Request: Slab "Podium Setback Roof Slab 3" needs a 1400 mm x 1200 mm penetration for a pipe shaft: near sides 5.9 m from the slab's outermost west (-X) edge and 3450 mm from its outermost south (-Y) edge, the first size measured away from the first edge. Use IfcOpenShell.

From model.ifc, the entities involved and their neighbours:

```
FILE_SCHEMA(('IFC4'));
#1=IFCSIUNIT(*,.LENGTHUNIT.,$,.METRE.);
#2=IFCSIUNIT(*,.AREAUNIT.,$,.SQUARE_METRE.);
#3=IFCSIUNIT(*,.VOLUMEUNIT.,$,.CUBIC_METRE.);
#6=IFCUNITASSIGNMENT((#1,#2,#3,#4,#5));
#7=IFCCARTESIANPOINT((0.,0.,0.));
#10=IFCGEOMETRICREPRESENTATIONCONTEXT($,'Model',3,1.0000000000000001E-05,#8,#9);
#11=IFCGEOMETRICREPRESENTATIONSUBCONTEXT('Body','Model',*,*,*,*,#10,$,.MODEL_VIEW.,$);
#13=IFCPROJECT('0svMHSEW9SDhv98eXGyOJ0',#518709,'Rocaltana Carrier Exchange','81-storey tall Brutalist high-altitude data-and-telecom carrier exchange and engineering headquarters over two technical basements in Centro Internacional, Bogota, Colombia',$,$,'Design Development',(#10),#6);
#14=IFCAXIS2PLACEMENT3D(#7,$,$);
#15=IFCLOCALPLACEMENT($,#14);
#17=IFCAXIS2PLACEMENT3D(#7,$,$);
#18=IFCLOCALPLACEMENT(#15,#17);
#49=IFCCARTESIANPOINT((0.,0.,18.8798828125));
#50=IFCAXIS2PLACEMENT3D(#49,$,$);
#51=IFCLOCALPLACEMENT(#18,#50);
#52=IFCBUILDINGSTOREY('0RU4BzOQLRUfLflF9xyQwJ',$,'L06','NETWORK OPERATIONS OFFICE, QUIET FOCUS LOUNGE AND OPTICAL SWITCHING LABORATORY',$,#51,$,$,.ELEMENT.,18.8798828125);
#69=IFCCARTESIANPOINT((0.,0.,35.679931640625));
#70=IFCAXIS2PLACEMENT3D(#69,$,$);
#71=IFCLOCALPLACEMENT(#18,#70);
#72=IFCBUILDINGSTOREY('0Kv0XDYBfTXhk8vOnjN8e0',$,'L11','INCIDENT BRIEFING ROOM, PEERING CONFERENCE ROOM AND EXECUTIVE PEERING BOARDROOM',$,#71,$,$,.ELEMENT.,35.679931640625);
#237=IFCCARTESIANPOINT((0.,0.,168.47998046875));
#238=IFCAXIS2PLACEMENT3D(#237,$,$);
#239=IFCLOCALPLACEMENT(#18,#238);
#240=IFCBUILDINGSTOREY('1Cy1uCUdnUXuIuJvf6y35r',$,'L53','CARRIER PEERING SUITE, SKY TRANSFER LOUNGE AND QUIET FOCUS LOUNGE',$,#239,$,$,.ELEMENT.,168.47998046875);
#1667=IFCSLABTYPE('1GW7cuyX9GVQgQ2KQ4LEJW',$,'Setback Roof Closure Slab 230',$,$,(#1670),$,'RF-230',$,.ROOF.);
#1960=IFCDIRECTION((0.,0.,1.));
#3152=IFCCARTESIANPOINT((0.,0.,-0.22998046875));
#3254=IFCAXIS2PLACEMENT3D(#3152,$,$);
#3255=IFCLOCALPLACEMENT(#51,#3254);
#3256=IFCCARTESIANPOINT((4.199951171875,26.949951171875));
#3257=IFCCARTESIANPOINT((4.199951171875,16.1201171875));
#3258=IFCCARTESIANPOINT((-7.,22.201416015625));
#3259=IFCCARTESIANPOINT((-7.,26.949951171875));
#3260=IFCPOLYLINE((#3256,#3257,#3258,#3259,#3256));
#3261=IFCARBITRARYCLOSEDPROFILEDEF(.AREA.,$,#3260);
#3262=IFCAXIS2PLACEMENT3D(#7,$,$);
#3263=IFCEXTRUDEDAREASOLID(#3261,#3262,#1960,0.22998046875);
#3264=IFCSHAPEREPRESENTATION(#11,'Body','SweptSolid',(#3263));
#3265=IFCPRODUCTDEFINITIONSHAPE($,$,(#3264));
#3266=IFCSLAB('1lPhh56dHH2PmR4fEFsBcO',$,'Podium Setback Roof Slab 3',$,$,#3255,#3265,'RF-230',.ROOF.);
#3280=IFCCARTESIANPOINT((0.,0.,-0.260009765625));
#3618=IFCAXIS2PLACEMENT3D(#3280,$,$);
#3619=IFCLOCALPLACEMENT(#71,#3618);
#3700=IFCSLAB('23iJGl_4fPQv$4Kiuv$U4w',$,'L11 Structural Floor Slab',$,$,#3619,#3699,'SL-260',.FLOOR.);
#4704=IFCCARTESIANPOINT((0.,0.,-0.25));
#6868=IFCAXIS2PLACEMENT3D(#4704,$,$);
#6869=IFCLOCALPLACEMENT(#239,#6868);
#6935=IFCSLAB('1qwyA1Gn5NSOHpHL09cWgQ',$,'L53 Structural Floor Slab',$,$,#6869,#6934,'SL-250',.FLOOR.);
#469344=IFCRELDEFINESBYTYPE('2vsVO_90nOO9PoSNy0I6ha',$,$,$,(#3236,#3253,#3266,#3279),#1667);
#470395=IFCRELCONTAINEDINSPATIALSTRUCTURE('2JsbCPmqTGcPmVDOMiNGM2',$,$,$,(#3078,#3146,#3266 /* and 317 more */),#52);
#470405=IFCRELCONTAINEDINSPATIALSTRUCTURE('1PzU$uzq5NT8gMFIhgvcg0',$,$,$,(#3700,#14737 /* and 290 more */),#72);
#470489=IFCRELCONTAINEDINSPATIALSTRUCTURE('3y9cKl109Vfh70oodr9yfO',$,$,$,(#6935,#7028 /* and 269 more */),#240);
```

```python
import numpy as np
import ifcopenshell
import ifcopenshell.api.feature
import ifcopenshell.api.geometry
import ifcopenshell.api.root
import ifcopenshell.geom
import ifcopenshell.util.placement
import ifcopenshell.util.representation
import ifcopenshell.util.shape
import ifcopenshell.util.unit

model = ifcopenshell.open("model.ifc")
unit_scale = ifcopenshell.util.unit.calculate_unit_scale(model)
settings = ifcopenshell.geom.settings()


def volume(element):
    """Net volume in cubic metres, openings subtracted."""
    shape = ifcopenshell.geom.create_shape(settings, element)
    return ifcopenshell.util.shape.get_volume(shape.geometry)


slab = model.by_id(3266)
before = volume(slab)

# Extent in the slab's own axes, in metres. The edges named are its -X and -Y sides.
slab_shape = ifcopenshell.geom.create_shape(settings, slab)
vertices = ifcopenshell.util.shape.get_vertices(slab_shape.geometry)
x_min, y_min, bottom = vertices.min(axis=0)
top = vertices[:, 2].max()

opening = ifcopenshell.api.root.create_entity(model, ifc_class="IfcOpeningElement", name="Pipe shaft opening", predefined_type="OPENING")
context = ifcopenshell.util.representation.get_context(model, "Model", "Body", "MODEL_VIEW")
width, depth = 1.4, 1.2
outline = [(0.0, 0.0), (width, 0.0), (width, depth), (0.0, depth), (0.0, 0.0)]
# Overshoot both faces by 50 mm so the cut is clean.
shape = ifcopenshell.api.geometry.add_slab_representation(
    model, context=context, depth=top - bottom + 0.1, polyline=outline
)
ifcopenshell.api.geometry.assign_representation(model, product=opening, representation=shape)

matrix = ifcopenshell.util.placement.get_local_placement(slab.ObjectPlacement)
matrix[:, 3] = matrix @ np.append(np.array([x_min + 5.9, y_min + 3.45, bottom - 0.05]) / unit_scale, 1.0)
ifcopenshell.api.geometry.edit_object_placement(model, product=opening, matrix=matrix, is_si=False)
ifcopenshell.api.feature.add_feature(model, feature=opening, element=slab)

after = volume(slab)

print(f"slab volume {before:.3f} -> {after:.3f} m3")

model.write("model-out.ifc")
```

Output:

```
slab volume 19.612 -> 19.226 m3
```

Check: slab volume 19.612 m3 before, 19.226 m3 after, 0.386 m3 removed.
